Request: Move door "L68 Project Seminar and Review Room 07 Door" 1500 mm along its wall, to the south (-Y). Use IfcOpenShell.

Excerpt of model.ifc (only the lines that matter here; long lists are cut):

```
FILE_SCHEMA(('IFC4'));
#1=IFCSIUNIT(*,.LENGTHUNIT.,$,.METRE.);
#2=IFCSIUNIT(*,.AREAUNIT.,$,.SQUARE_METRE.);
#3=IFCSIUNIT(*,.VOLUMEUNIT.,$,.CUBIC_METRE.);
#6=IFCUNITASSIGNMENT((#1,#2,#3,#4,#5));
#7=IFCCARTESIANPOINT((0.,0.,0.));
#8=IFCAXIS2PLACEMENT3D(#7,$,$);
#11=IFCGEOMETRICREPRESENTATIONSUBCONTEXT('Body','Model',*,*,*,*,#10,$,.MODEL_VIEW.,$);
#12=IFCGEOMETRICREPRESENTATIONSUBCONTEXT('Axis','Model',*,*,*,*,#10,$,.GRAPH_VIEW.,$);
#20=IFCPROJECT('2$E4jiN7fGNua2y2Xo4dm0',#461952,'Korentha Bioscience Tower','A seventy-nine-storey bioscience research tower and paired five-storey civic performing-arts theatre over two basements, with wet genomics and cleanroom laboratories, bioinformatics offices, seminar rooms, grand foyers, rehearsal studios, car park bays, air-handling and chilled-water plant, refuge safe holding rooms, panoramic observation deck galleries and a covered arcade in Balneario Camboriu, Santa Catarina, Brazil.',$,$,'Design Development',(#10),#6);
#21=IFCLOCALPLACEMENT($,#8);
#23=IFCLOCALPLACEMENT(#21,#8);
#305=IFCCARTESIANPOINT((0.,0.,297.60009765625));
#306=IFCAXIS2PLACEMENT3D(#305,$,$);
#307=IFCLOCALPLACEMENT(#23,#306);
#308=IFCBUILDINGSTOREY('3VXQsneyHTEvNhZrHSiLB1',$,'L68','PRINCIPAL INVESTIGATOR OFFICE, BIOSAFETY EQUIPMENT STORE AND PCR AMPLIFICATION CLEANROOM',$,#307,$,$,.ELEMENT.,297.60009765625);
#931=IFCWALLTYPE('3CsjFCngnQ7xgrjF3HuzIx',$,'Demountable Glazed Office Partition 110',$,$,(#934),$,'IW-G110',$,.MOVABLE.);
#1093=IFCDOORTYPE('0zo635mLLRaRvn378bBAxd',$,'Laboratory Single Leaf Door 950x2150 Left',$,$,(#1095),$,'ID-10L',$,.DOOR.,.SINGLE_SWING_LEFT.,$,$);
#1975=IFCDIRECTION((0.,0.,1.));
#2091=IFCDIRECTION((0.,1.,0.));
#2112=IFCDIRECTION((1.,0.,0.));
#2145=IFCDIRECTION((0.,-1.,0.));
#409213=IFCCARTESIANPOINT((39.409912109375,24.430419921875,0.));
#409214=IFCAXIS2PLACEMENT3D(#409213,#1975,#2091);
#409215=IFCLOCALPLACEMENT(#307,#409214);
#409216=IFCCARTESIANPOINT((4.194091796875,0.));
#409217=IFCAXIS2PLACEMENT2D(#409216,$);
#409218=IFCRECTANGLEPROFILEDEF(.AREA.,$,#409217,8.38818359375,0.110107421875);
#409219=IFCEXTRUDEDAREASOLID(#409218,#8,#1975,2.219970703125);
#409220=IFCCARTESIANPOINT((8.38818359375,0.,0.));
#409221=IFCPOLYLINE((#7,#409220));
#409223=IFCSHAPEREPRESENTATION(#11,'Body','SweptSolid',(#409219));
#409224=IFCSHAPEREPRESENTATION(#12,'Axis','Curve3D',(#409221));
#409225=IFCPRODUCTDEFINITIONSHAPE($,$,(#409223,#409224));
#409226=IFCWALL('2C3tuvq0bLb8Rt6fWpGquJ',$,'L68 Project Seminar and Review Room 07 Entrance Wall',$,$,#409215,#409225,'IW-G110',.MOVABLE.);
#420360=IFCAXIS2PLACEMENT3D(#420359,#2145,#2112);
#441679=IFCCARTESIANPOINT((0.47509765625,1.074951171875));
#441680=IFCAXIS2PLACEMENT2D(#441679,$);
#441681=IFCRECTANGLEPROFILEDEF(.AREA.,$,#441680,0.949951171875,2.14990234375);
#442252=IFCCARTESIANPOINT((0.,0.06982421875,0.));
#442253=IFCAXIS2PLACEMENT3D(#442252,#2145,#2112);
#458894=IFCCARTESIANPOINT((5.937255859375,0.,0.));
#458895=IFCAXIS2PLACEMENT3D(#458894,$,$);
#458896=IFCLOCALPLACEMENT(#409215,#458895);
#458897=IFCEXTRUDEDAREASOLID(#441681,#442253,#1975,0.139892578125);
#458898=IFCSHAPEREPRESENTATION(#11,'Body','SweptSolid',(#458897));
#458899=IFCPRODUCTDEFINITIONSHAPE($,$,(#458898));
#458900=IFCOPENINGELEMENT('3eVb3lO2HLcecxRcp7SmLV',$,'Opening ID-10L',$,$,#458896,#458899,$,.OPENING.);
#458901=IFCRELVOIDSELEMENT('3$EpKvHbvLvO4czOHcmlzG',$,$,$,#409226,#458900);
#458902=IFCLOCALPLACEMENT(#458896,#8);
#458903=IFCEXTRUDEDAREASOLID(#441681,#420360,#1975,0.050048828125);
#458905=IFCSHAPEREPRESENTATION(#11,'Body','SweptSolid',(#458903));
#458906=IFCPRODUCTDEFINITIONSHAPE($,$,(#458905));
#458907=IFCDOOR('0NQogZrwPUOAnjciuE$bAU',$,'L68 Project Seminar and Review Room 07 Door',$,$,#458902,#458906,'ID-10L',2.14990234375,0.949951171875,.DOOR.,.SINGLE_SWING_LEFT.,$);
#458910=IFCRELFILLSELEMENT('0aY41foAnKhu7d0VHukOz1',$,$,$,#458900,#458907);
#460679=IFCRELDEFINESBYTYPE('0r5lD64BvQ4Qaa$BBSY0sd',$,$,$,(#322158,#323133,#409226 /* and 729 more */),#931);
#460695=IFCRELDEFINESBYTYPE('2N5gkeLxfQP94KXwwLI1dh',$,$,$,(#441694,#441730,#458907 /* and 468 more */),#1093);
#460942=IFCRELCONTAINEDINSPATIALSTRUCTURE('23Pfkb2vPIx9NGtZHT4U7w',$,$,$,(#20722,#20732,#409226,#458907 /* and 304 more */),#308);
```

```python
import ifcopenshell
import ifcopenshell.api.geometry
import ifcopenshell.util.placement

model = ifcopenshell.open("model.ifc")

door = model.by_guid("0NQogZrwPUOAnjciuE$bAU")
opening = door.FillsVoids[0].RelatingOpeningElement
wall = opening.VoidsElements[0].RelatingBuildingElement

wall_matrix = ifcopenshell.util.placement.get_local_placement(wall.ObjectPlacement)
shift = wall_matrix[:3, 0] * -1.5
before = ifcopenshell.util.placement.get_local_placement(door.ObjectPlacement)[:3, 3].copy()

# The door is placed relative to its opening, so it follows when the opening moves.
matrix = ifcopenshell.util.placement.get_local_placement(opening.ObjectPlacement)
matrix[:3, 3] += shift
ifcopenshell.api.geometry.edit_object_placement(
    model, product=opening, matrix=matrix, is_si=False, should_transform_children=True
)

after = ifcopenshell.util.placement.get_local_placement(door.ObjectPlacement)[:3, 3]
print("door moved by", (after - before).round(3) + 0.0)

model.write("model_rev.ifc")
```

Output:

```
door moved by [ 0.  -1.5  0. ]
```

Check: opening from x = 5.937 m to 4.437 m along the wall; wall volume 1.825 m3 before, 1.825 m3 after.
